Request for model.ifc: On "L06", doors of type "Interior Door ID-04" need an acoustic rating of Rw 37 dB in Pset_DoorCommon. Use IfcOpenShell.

First a look at what the model holds.

```python
import ifcopenshell
import ifcopenshell.util.element

model = ifcopenshell.open("model.ifc")
print(model.schema)
storey = next(s for s in model.by_type("IfcBuildingStorey") if s.Name == "L06")
doors = [e for e in ifcopenshell.util.element.get_decomposition(storey) if e.is_a("IfcDoor")]
seen = {}
for e in doors:
    element_type = ifcopenshell.util.element.get_type(e)
    key = (element_type.Name if element_type != e and element_type else None, ifcopenshell.util.element.get_pset(e, "Pset_DoorCommon", "AcousticRating"))
    seen[key] = seen.get(key, 0) + 1
for (name, value), count in sorted(seen.items(), key=str):
    print(count, "x", name, "|", value)
```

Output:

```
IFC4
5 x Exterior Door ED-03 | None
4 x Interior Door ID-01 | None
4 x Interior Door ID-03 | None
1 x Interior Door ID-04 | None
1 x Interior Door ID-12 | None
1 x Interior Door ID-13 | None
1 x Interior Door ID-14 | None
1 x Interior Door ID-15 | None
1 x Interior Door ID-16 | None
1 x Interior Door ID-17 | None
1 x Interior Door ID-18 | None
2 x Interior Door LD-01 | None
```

```python
import ifcopenshell
import ifcopenshell.api.pset
import ifcopenshell.util.element

model = ifcopenshell.open("model.ifc")

storey = next(s for s in model.by_type("IfcBuildingStorey") if s.Name == "L06")
doors = [e for e in ifcopenshell.util.element.get_decomposition(storey) if e.is_a("IfcDoor")]

count = 0
for e in doors:
    element_type = ifcopenshell.util.element.get_type(e)
    if element_type in (None, e) or element_type.Name != "Interior Door ID-04":
        continue
    # add_pset returns the element's existing set when there is one.
    pset = ifcopenshell.api.pset.add_pset(model, product=e, name="Pset_DoorCommon")
    ifcopenshell.api.pset.edit_pset(model, pset=pset, properties={"AcousticRating": "Rw 37 dB"})
    count += 1

print(count, "doors updated")

model.write("model_rev.ifc")
```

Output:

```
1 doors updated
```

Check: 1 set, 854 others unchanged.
